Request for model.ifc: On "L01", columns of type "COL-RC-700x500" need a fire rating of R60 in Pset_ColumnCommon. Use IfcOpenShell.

First a look at what the model holds.

```python
import ifcopenshell
import ifcopenshell.util.element

model = ifcopenshell.open("model.ifc")
print(model.schema)
storey = next(s for s in model.by_type("IfcBuildingStorey") if s.Name == "L01")
columns = [e for e in ifcopenshell.util.element.get_decomposition(storey) if e.is_a("IfcColumn")]
seen = {}
for e in columns:
    element_type = ifcopenshell.util.element.get_type(e)
    key = (element_type.Name if element_type != e and element_type else None, ifcopenshell.util.element.get_pset(e, "Pset_ColumnCommon", "FireRating"))
    seen[key] = seen.get(key, 0) + 1
for (name, value), count in sorted(seen.items(), key=str):
    print(count, "x", name, "|", value)
```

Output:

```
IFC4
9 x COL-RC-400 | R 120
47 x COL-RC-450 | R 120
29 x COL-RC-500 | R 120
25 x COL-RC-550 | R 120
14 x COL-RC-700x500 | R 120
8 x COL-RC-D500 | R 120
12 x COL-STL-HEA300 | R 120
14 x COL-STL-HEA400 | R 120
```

```python
import ifcopenshell
import ifcopenshell.api.pset
import ifcopenshell.util.element

model = ifcopenshell.open("model.ifc")

storey = next(s for s in model.by_type("IfcBuildingStorey") if s.Name == "L01")
columns = [e for e in ifcopenshell.util.element.get_decomposition(storey) if e.is_a("IfcColumn")]

count = 0
for e in columns:
    element_type = ifcopenshell.util.element.get_type(e)
    if element_type in (None, e) or element_type.Name != "COL-RC-700x500":
        continue
    # add_pset returns the element's existing set when there is one.
    pset = ifcopenshell.api.pset.add_pset(model, product=e, name="Pset_ColumnCommon")
    ifcopenshell.api.pset.edit_pset(model, pset=pset, properties={"FireRating": "R60"})
    count += 1

print(count, "columns updated")

model.write("model_updated.ifc")
```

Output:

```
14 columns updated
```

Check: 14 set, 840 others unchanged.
